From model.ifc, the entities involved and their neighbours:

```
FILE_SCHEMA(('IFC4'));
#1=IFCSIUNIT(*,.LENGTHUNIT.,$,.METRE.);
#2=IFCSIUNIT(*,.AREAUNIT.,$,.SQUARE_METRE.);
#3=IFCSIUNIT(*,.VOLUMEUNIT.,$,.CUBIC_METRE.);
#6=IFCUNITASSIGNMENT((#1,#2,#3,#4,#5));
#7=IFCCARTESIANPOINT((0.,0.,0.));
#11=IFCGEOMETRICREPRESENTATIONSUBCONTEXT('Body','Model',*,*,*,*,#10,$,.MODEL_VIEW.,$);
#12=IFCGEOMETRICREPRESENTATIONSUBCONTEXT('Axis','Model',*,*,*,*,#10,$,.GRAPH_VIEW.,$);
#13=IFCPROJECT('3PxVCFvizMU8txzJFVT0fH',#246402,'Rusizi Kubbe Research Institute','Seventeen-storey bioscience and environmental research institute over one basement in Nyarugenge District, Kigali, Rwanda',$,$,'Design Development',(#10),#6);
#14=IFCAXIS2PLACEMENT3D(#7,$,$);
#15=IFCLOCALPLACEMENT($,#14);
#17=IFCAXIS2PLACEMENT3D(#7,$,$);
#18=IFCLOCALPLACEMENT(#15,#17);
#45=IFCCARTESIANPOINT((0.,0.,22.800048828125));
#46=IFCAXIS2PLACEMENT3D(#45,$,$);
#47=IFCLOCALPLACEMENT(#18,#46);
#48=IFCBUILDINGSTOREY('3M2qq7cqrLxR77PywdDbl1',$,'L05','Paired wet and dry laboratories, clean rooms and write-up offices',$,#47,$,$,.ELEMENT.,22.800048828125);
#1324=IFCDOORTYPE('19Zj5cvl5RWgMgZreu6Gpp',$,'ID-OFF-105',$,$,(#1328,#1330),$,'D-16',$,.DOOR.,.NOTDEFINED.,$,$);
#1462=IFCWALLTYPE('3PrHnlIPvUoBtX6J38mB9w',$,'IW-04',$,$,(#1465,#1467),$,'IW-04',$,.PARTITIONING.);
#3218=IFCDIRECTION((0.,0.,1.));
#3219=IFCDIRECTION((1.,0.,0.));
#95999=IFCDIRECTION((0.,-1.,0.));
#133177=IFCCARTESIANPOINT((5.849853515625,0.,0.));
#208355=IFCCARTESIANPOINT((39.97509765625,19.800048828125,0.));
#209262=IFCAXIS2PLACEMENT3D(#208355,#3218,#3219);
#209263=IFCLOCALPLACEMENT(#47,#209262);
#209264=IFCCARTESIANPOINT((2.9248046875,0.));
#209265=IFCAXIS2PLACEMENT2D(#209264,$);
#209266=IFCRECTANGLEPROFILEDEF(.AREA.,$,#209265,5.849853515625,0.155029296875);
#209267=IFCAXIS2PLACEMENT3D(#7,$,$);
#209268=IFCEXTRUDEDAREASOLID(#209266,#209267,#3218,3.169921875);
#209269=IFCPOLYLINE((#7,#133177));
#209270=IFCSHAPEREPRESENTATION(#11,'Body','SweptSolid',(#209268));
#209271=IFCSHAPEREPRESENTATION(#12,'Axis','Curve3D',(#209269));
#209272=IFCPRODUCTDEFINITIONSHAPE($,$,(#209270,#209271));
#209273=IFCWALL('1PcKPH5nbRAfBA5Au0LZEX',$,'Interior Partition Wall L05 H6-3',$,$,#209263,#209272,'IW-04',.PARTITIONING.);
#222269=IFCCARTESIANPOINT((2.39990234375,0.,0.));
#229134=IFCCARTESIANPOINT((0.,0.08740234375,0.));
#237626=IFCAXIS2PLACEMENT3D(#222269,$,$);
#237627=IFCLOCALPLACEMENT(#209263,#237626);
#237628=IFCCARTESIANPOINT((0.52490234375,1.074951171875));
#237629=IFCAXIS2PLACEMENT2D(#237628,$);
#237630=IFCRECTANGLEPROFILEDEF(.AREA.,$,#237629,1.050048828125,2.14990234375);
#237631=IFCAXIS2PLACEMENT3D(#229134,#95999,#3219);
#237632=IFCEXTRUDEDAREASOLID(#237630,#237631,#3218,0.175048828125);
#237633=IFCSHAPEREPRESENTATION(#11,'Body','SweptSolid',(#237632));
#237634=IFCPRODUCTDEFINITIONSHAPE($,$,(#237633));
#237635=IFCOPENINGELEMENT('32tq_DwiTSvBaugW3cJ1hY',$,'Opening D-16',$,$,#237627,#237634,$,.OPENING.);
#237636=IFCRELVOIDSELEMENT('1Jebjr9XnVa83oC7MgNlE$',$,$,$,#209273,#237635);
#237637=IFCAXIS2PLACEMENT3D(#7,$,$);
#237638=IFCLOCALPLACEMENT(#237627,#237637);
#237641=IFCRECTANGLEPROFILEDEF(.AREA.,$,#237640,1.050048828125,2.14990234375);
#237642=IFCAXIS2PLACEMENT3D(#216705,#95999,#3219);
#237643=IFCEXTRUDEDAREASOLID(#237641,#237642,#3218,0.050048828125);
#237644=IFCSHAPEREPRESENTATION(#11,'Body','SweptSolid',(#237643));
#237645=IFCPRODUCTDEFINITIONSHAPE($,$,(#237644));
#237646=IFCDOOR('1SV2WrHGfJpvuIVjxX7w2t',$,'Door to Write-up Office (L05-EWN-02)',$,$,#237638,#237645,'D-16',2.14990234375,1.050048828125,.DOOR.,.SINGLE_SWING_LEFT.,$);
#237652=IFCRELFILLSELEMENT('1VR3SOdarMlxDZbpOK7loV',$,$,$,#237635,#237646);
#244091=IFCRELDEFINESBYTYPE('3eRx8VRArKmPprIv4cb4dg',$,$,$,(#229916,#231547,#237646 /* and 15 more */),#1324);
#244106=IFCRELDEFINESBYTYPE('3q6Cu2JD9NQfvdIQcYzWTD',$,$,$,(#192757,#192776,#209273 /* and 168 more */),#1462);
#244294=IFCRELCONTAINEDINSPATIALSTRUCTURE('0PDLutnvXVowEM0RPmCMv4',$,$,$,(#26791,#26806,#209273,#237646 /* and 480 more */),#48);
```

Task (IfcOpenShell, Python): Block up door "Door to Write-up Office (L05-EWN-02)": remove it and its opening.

```python
import ifcopenshell
import ifcopenshell.api.feature
import ifcopenshell.api.root
import ifcopenshell.geom
import ifcopenshell.util.shape

model = ifcopenshell.open("model.ifc")
settings = ifcopenshell.geom.settings()


def volume(element):
    """Net volume in cubic metres, openings subtracted."""
    shape = ifcopenshell.geom.create_shape(settings, element)
    return ifcopenshell.util.shape.get_volume(shape.geometry)


door = model.by_guid("1SV2WrHGfJpvuIVjxX7w2t")
opening = door.FillsVoids[0].RelatingOpeningElement
wall = opening.VoidsElements[0].RelatingBuildingElement
before = volume(wall)

ifcopenshell.api.root.remove_product(model, product=door)
ifcopenshell.api.feature.remove_feature(model, feature=opening)

after = volume(wall)

print(f"wall volume {before:.3f} -> {after:.3f} m3")

model.write("model-out.ifc")
```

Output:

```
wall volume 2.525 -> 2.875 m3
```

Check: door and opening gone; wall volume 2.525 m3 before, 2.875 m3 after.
